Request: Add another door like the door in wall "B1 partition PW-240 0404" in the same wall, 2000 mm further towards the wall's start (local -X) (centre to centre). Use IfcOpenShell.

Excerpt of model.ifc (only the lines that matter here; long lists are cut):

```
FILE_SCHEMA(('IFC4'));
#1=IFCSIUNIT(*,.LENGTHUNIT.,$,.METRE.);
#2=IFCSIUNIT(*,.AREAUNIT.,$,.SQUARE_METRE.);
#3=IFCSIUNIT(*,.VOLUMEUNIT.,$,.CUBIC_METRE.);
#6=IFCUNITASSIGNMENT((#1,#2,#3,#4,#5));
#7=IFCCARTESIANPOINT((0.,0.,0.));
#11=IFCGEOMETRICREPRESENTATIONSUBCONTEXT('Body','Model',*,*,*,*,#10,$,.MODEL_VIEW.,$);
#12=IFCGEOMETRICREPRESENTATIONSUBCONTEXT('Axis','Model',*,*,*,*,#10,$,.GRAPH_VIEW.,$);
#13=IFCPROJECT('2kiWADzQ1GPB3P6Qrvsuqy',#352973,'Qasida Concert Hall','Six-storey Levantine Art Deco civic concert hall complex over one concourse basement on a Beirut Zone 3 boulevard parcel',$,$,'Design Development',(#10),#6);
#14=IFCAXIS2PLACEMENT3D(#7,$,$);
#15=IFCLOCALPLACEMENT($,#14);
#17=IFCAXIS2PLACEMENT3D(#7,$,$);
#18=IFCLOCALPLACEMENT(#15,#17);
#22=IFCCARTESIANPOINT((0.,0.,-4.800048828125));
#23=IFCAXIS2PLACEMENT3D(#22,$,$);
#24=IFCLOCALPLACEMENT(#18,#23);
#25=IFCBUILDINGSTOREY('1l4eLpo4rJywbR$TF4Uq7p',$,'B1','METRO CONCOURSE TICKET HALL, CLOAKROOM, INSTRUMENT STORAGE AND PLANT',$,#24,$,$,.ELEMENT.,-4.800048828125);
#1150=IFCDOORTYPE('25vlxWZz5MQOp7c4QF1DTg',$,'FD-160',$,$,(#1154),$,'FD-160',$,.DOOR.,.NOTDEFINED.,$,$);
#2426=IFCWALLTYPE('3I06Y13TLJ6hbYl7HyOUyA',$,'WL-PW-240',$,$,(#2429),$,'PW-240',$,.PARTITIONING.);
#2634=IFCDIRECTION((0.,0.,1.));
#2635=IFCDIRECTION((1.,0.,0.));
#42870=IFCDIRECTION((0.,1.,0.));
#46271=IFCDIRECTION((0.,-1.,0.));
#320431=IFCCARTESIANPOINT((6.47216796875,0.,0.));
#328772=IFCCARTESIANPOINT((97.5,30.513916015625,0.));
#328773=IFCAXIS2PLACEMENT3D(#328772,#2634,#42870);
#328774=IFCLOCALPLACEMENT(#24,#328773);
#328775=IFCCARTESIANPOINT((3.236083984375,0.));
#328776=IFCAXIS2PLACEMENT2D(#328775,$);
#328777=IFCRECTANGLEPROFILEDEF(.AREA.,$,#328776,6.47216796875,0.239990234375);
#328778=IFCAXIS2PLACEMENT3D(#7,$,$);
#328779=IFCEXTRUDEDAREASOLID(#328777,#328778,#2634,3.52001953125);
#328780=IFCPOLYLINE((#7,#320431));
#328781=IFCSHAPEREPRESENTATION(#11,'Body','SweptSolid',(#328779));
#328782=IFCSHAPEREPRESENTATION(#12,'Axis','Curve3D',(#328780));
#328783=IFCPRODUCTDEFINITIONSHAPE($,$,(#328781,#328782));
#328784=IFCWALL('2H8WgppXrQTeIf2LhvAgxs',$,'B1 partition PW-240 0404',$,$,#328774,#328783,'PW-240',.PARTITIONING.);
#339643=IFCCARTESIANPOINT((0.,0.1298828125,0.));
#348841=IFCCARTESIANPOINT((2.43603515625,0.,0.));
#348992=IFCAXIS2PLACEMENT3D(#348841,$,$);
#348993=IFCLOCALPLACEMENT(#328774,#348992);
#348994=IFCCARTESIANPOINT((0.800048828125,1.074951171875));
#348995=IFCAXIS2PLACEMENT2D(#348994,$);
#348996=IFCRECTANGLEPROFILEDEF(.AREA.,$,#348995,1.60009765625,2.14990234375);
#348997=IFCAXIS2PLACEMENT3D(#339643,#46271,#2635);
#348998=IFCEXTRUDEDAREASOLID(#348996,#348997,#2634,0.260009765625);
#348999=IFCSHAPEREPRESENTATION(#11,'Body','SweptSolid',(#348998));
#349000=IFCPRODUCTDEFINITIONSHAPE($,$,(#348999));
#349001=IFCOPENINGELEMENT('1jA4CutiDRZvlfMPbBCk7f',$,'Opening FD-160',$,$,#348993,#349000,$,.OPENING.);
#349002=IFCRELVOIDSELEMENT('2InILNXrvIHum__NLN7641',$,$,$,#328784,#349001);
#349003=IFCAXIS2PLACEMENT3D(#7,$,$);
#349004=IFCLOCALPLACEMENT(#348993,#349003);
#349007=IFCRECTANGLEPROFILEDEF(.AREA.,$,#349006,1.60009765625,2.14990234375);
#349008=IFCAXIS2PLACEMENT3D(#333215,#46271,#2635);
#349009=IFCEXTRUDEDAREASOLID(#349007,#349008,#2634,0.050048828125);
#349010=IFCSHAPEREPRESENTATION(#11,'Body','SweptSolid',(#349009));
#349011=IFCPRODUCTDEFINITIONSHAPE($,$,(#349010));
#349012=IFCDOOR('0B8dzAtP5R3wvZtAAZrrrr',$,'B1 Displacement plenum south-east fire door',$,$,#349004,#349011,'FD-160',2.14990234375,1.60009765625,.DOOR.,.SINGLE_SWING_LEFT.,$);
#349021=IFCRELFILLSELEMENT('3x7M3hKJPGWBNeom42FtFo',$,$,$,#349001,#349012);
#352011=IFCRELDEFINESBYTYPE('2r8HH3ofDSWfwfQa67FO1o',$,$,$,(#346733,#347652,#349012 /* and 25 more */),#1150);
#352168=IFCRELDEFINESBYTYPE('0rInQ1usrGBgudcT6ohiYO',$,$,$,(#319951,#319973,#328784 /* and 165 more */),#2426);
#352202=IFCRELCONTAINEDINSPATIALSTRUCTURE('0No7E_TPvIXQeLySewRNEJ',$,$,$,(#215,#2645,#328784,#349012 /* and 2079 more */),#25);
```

```python
import ifcopenshell
import ifcopenshell.api.feature
import ifcopenshell.api.geometry
import ifcopenshell.api.root
import ifcopenshell.geom
import ifcopenshell.util.element
import ifcopenshell.util.placement
import ifcopenshell.util.shape
import ifcopenshell.util.unit

model = ifcopenshell.open("model.ifc")
unit_scale = ifcopenshell.util.unit.calculate_unit_scale(model)
settings = ifcopenshell.geom.settings()


def volume(element):
    """Net volume in cubic metres, openings subtracted."""
    shape = ifcopenshell.geom.create_shape(settings, element)
    return ifcopenshell.util.shape.get_volume(shape.geometry)


door = model.by_guid("0B8dzAtP5R3wvZtAAZrrrr")
opening = door.FillsVoids[0].RelatingOpeningElement
wall = opening.VoidsElements[0].RelatingBuildingElement
before = volume(wall)
shift = ifcopenshell.util.placement.get_local_placement(wall.ObjectPlacement)[:3, 0] * -2 / unit_scale

# copy_class copies the void relationship, type, container and properties, but no geometry.
new_opening = ifcopenshell.api.root.copy_class(model, product=opening)
new_opening.Representation = ifcopenshell.util.element.copy_deep(
    model, opening.Representation, exclude=["IfcGeometricRepresentationContext", "IfcRepresentationMap"]
)
new_door = ifcopenshell.api.root.copy_class(model, product=door)
new_door.Representation = ifcopenshell.util.element.copy_deep(
    model, door.Representation, exclude=["IfcGeometricRepresentationContext", "IfcRepresentationMap"]
)
new_door.Tag = None
ifcopenshell.api.feature.add_filling(model, opening=new_opening, element=new_door)

for old, new in ((opening, new_opening), (door, new_door)):
    matrix = ifcopenshell.util.placement.get_local_placement(old.ObjectPlacement)
    matrix[:3, 3] += shift
    ifcopenshell.api.geometry.edit_object_placement(model, product=new, matrix=matrix, is_si=False)

after = volume(wall)

print(f"wall volume {before:.3f} -> {after:.3f} m3")

model.write("model_updated.ifc")
```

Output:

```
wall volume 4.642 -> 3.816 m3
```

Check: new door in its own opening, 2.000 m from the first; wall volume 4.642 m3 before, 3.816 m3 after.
